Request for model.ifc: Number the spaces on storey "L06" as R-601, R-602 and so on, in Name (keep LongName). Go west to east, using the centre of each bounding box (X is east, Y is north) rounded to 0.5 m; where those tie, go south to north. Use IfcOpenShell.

First a look at what the model holds.

```python
import ifcopenshell
import ifcopenshell.util.element
import ifcopenshell.util.placement

model = ifcopenshell.open("model.ifc")
print(model.schema)
storey = next(s for s in model.by_type("IfcBuildingStorey") if s.Name == "L06")
spaces = [e for e in ifcopenshell.util.element.get_decomposition(storey) if e.is_a("IfcSpace")]
for e in sorted(spaces, key=lambda e: e.id()):
    origin = ifcopenshell.util.placement.get_local_placement(e.ObjectPlacement)[:3, 3]
    print(e.id(), e.Name, e.LongName, origin.round(2) + 0.0, sep=" | ")
```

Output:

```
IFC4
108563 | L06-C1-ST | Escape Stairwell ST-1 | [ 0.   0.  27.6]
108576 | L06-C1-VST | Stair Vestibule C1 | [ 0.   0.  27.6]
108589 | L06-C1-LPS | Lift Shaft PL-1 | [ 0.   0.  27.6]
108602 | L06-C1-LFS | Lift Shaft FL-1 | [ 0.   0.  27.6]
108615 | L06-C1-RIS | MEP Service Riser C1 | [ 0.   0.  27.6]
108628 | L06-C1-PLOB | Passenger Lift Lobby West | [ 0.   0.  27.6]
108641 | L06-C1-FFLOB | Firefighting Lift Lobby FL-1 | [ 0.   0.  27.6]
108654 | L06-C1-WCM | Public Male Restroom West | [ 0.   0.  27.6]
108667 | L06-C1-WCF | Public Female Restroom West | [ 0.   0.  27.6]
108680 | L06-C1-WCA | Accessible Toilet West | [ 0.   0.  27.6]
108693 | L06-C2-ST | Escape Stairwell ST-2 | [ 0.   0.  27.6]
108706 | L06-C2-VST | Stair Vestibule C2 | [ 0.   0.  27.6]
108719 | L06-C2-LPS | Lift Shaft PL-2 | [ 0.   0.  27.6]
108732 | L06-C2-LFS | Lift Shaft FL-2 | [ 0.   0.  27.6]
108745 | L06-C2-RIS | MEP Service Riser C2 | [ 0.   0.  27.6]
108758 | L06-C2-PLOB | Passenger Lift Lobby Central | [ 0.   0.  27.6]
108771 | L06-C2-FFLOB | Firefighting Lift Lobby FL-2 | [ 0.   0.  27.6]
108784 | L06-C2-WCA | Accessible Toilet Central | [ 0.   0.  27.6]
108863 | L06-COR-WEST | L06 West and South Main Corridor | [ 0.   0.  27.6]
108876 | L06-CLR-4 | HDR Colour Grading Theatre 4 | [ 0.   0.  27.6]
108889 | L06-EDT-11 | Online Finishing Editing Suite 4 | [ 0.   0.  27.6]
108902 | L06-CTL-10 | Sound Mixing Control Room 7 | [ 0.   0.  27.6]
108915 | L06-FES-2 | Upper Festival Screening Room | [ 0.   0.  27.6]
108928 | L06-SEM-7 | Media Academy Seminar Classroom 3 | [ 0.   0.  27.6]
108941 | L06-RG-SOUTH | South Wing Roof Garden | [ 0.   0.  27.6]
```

```python
import ifcopenshell
import ifcopenshell.geom
import ifcopenshell.util.element
import ifcopenshell.util.shape

model = ifcopenshell.open("model.ifc")
settings = ifcopenshell.geom.settings()
settings.set("use-world-coords", True)


def centre(element):
    shape = ifcopenshell.geom.create_shape(settings, element)
    return ifcopenshell.util.shape.get_bbox_centroid(shape.geometry)


storey = next(s for s in model.by_type("IfcBuildingStorey") if s.Name == "L06")
spaces = [e for e in ifcopenshell.util.element.get_decomposition(storey) if e.is_a("IfcSpace")]

# Insertion points can sit at a corner or the storey origin, so sort by the geometry (in metres).
centres = {e: centre(e) for e in spaces}
spaces.sort(key=lambda e: (round(centres[e][0] / 0.5), centres[e][1]))

for i, e in enumerate(spaces, start=1):
    number = f"R-6{i:02d}"
    e.Name = number
    print(e.id(), number)

model.write("model_rev.ifc")
```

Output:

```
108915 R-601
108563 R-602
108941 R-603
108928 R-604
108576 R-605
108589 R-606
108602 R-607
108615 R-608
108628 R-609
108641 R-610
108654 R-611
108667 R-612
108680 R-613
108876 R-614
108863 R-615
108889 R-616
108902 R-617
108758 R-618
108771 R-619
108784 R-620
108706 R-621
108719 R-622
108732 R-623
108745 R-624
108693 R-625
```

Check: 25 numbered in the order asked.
